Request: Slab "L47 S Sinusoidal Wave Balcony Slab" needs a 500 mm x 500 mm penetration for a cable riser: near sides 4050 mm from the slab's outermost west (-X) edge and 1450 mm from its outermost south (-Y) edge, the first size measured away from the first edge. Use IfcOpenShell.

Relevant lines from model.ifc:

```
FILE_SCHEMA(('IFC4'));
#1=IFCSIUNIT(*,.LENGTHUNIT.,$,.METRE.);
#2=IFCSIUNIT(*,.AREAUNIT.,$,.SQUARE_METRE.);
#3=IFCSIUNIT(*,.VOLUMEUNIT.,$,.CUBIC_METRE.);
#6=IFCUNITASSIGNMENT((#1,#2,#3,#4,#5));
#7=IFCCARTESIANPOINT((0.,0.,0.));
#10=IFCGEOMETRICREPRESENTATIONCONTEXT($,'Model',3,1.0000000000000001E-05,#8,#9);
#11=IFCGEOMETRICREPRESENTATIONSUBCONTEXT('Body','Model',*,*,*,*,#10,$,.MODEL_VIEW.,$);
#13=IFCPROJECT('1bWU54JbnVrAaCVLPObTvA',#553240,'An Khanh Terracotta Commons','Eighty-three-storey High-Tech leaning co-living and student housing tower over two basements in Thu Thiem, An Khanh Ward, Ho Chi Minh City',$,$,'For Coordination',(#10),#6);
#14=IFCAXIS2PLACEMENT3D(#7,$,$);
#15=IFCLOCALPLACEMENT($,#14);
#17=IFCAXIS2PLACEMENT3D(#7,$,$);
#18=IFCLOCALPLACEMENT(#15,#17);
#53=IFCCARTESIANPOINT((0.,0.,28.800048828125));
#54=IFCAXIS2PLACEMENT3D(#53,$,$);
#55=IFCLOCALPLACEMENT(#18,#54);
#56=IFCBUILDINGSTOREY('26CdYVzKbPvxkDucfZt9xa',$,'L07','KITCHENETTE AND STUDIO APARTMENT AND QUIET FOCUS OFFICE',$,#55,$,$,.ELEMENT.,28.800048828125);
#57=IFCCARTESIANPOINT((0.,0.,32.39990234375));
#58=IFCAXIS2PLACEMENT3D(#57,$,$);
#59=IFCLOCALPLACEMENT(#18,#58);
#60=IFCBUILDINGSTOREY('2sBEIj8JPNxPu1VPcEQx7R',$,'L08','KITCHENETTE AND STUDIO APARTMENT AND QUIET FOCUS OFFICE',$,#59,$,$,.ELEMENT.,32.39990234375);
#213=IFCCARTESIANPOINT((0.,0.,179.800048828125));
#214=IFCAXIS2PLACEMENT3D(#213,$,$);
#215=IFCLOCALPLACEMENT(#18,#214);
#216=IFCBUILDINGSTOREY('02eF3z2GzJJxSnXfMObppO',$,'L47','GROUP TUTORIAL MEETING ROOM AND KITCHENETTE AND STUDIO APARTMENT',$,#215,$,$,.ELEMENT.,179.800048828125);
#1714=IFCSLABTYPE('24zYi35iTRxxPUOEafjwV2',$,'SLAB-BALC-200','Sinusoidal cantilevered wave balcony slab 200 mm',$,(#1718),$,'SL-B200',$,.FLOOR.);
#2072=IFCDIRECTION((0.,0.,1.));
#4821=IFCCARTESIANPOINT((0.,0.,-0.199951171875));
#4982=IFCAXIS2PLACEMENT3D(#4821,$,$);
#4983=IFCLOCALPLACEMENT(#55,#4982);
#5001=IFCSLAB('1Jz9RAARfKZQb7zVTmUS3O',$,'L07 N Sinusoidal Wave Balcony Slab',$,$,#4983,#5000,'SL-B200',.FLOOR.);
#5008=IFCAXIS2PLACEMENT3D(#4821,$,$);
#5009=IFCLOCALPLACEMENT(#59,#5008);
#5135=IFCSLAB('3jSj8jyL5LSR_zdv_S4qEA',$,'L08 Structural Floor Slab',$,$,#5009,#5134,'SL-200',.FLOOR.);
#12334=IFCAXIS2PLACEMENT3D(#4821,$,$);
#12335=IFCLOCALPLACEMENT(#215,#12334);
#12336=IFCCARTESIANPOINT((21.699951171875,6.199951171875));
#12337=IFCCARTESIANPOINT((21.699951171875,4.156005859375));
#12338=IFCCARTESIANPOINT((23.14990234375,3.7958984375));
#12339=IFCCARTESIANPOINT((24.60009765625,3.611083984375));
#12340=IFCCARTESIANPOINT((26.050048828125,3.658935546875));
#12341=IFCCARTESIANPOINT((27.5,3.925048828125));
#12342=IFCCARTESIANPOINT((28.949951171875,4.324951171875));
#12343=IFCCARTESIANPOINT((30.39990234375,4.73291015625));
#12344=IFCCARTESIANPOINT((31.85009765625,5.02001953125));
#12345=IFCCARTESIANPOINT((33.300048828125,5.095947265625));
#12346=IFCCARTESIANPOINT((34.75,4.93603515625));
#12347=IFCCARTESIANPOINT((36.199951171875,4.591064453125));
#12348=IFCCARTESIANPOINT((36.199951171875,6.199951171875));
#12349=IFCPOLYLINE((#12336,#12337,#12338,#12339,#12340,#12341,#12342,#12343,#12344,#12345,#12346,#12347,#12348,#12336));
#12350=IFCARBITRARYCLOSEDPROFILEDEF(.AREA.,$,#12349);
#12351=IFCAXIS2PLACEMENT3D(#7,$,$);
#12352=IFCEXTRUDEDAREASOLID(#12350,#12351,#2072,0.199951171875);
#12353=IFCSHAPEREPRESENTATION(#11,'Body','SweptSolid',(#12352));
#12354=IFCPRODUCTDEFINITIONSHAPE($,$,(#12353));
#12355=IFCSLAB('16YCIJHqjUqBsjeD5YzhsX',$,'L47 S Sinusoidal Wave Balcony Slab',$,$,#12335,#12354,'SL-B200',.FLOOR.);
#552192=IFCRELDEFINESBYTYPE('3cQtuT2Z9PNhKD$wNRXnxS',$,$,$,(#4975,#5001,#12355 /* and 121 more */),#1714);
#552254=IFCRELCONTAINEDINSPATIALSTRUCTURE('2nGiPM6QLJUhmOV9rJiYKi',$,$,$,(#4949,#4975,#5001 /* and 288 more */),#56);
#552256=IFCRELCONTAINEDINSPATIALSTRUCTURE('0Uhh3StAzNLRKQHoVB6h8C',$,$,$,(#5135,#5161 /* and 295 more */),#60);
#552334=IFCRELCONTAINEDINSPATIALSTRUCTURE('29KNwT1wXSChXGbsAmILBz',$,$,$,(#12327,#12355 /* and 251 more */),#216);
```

```python
import numpy as np
import ifcopenshell
import ifcopenshell.api.feature
import ifcopenshell.api.geometry
import ifcopenshell.api.root
import ifcopenshell.geom
import ifcopenshell.util.placement
import ifcopenshell.util.representation
import ifcopenshell.util.shape
import ifcopenshell.util.unit

model = ifcopenshell.open("model.ifc")
unit_scale = ifcopenshell.util.unit.calculate_unit_scale(model)
settings = ifcopenshell.geom.settings()


def volume(element):
    """Net volume in cubic metres, openings subtracted."""
    shape = ifcopenshell.geom.create_shape(settings, element)
    return ifcopenshell.util.shape.get_volume(shape.geometry)


slab = model.by_guid("16YCIJHqjUqBsjeD5YzhsX")
before = volume(slab)

# Extent in the slab's own axes, in metres. The edges named are its -X and -Y sides.
slab_shape = ifcopenshell.geom.create_shape(settings, slab)
vertices = ifcopenshell.util.shape.get_vertices(slab_shape.geometry)
x_min, y_min, bottom = vertices.min(axis=0)
top = vertices[:, 2].max()

opening = ifcopenshell.api.root.create_entity(model, ifc_class="IfcOpeningElement", name="Cable riser opening", predefined_type="OPENING")
context = ifcopenshell.util.representation.get_context(model, "Model", "Body", "MODEL_VIEW")
width, depth = 0.5, 0.5
outline = [(0.0, 0.0), (width, 0.0), (width, depth), (0.0, depth), (0.0, 0.0)]
# Overshoot both faces by 50 mm so the cut is clean.
shape = ifcopenshell.api.geometry.add_slab_representation(
    model, context=context, depth=top - bottom + 0.1, polyline=outline
)
ifcopenshell.api.geometry.assign_representation(model, product=opening, representation=shape)

matrix = ifcopenshell.util.placement.get_local_placement(slab.ObjectPlacement)
matrix[:, 3] = matrix @ np.append(np.array([x_min + 4.05, y_min + 1.45, bottom - 0.05]) / unit_scale, 1.0)
ifcopenshell.api.geometry.edit_object_placement(model, product=opening, matrix=matrix, is_si=False)
ifcopenshell.api.feature.add_feature(model, feature=opening, element=slab)

after = volume(slab)

print(f"slab volume {before:.3f} -> {after:.3f} m3")

model.write("model-out.ifc")
```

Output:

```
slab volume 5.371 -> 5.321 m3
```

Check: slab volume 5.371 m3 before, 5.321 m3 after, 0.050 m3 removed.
